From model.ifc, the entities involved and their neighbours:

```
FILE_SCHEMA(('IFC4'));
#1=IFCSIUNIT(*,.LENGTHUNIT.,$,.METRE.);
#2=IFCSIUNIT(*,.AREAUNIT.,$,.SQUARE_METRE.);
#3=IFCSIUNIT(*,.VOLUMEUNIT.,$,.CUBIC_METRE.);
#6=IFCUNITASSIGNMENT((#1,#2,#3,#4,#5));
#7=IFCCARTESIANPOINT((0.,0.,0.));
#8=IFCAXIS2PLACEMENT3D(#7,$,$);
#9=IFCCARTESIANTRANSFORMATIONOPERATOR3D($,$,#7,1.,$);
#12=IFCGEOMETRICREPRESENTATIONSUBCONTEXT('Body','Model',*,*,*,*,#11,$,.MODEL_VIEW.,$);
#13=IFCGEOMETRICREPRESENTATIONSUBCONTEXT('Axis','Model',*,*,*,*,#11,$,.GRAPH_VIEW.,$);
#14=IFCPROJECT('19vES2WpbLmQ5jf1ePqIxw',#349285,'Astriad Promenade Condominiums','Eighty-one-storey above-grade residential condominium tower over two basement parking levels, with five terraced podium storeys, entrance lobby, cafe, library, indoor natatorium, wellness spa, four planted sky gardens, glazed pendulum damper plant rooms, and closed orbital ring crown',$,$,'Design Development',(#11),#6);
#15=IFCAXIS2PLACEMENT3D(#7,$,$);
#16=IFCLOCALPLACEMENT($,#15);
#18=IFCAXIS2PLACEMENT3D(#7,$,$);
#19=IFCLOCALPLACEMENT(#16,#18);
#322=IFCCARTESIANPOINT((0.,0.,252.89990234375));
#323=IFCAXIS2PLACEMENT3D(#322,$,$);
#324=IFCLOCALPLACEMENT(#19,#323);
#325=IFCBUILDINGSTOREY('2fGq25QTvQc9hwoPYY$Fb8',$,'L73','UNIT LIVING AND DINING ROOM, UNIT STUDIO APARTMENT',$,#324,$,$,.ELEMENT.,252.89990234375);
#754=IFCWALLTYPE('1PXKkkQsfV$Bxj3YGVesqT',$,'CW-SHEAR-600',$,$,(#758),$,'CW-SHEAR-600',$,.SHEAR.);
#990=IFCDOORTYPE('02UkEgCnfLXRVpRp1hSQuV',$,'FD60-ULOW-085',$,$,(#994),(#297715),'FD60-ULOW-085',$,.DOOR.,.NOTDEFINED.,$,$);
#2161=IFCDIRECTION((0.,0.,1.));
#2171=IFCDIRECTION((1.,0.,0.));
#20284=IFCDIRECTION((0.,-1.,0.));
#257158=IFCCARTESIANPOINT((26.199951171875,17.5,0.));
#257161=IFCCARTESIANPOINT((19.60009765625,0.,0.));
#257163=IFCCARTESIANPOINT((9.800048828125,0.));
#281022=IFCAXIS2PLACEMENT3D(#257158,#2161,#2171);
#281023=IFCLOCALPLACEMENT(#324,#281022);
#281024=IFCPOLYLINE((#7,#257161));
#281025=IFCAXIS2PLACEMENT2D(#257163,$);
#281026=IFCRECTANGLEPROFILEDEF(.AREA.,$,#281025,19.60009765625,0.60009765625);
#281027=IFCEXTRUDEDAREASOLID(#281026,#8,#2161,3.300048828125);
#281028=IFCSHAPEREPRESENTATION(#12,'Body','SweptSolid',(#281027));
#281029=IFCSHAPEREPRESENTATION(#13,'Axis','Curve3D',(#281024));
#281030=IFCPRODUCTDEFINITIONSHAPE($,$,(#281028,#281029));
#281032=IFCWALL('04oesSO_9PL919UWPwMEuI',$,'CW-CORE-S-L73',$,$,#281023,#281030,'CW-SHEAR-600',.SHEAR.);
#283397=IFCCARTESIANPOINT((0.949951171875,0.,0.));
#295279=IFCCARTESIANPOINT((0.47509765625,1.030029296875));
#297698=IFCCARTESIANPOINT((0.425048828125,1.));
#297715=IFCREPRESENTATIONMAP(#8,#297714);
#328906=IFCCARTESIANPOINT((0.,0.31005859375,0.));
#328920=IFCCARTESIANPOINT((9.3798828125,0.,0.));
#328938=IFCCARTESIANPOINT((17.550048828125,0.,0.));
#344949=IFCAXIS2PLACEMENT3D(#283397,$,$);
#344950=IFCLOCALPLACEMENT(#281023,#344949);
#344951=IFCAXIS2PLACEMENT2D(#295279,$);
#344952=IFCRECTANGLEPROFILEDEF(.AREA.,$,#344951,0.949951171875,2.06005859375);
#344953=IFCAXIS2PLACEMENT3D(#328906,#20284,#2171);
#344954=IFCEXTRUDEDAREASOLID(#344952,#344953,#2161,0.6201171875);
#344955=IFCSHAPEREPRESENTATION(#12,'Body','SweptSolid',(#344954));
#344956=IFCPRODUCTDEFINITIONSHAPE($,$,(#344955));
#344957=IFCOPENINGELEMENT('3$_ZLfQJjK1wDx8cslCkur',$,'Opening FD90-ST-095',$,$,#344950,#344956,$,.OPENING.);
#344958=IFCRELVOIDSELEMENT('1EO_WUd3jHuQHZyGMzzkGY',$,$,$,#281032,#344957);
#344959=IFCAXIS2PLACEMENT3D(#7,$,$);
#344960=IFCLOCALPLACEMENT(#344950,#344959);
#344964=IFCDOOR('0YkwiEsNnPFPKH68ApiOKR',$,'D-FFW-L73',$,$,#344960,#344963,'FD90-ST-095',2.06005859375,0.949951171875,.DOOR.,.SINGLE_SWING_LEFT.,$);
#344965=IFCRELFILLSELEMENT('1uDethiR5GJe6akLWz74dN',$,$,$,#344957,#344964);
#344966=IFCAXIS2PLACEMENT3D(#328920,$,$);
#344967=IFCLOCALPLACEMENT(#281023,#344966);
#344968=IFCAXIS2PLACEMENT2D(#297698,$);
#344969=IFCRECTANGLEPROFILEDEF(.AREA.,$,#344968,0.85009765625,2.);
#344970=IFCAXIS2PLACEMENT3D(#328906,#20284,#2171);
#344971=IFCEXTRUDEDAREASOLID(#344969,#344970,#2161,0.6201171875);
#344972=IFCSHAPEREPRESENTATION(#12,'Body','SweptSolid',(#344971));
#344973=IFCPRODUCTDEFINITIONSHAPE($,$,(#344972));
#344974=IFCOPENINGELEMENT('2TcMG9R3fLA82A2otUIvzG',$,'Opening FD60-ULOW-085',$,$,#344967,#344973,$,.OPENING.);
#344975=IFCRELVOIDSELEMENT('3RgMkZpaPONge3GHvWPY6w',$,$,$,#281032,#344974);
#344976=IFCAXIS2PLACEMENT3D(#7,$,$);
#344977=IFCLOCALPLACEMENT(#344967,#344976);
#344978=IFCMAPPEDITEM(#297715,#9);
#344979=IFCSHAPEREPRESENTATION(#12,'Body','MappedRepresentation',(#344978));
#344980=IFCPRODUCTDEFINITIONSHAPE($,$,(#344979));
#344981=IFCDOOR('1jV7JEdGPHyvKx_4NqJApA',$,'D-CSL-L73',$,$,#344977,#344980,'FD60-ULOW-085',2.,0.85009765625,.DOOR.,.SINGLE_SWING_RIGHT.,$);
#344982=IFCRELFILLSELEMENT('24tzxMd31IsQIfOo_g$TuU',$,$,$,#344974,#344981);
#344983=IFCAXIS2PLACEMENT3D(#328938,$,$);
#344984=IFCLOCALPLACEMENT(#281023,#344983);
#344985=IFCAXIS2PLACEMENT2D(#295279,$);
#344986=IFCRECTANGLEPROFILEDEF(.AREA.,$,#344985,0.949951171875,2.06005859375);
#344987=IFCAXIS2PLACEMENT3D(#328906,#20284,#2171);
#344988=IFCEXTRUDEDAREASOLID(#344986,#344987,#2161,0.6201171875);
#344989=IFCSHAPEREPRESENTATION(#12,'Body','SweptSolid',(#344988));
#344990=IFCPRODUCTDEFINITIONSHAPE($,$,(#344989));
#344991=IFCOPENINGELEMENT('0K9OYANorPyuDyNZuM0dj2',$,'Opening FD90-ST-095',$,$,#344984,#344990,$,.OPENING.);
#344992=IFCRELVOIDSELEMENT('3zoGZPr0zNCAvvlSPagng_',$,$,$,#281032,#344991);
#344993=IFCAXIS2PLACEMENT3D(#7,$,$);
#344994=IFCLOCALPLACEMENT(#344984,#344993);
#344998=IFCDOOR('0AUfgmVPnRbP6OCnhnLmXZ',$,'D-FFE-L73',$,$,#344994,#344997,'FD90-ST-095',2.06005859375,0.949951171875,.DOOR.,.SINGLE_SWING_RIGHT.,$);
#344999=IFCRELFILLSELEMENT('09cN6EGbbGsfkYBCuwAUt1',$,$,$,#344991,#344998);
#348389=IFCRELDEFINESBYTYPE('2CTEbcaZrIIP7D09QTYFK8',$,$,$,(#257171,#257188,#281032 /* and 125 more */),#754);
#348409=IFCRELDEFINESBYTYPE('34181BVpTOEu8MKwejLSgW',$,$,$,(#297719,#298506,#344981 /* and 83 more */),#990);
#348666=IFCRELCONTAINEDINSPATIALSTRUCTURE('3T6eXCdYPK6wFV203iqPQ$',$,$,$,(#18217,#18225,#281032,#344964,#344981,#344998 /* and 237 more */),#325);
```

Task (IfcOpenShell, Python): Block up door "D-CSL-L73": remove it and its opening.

```python
import ifcopenshell
import ifcopenshell.api.feature
import ifcopenshell.api.root
import ifcopenshell.geom
import ifcopenshell.util.shape

model = ifcopenshell.open("model.ifc")
settings = ifcopenshell.geom.settings()


def volume(element):
    """Net volume in cubic metres, openings subtracted."""
    shape = ifcopenshell.geom.create_shape(settings, element)
    return ifcopenshell.util.shape.get_volume(shape.geometry)


door = model.by_guid("1jV7JEdGPHyvKx_4NqJApA")
opening = door.FillsVoids[0].RelatingOpeningElement
wall = opening.VoidsElements[0].RelatingBuildingElement
before = volume(wall)

ifcopenshell.api.root.remove_product(model, product=door)
ifcopenshell.api.feature.remove_feature(model, feature=opening)

after = volume(wall)

print(f"wall volume {before:.3f} -> {after:.3f} m3")

model.write("model-out.ifc")
```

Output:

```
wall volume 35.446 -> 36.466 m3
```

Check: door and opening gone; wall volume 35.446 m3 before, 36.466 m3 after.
